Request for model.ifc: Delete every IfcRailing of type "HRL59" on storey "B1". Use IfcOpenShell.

First a look at what the model holds.

```python
import ifcopenshell
import ifcopenshell.util.element

model = ifcopenshell.open("model.ifc")
print(model.schema)
storey = next(s for s in model.by_type("IfcBuildingStorey") if s.Name == "B1")
railings = [e for e in ifcopenshell.util.element.get_decomposition(storey) if e.is_a("IfcRailing")]
seen = {}
for e in railings:
    element_type = ifcopenshell.util.element.get_type(e)
    name = element_type.Name if element_type not in (None, e) else None
    seen[name] = seen.get(name, 0) + 1
for name, count in sorted(seen.items(), key=str):
    print(count, "x", name)
```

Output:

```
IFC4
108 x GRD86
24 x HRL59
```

```python
import ifcopenshell
import ifcopenshell.api.root
import ifcopenshell.util.element

model = ifcopenshell.open("model.ifc")

storey = next(s for s in model.by_type("IfcBuildingStorey") if s.Name == "B1")
railings = [e for e in ifcopenshell.util.element.get_decomposition(storey) if e.is_a("IfcRailing")]
targets = [e for e in railings if (t := ifcopenshell.util.element.get_type(e)) not in (None, e) and t.Name == "HRL59"]

for e in targets:
    ifcopenshell.api.root.remove_product(model, product=e)
print(len(targets), "removed")

model.write("model_updated.ifc")
```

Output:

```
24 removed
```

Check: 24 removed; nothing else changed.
